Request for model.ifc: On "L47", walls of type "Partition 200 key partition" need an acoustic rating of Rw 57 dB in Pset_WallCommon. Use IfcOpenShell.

First a look at what the model holds.

```python
import ifcopenshell
import ifcopenshell.util.element

model = ifcopenshell.open("model.ifc")
print(model.schema)
storey = next(s for s in model.by_type("IfcBuildingStorey") if s.Name == "L47")
walls = [e for e in ifcopenshell.util.element.get_decomposition(storey) if e.is_a("IfcWall")]
seen = {}
for e in walls:
    element_type = ifcopenshell.util.element.get_type(e)
    key = (element_type.Name if element_type != e and element_type else None, ifcopenshell.util.element.get_pset(e, "Pset_WallCommon", "AcousticRating"))
    seen[key] = seen.get(key, 0) + 1
for (name, value), count in sorted(seen.items(), key=str):
    print(count, "x", name, "|", value)
```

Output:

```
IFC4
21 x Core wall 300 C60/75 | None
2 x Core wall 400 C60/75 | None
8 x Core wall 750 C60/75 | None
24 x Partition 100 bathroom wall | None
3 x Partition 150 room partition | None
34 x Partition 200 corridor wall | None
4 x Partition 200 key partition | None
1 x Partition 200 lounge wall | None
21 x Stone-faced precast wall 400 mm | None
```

```python
import ifcopenshell
import ifcopenshell.api.pset
import ifcopenshell.util.element

model = ifcopenshell.open("model.ifc")

storey = next(s for s in model.by_type("IfcBuildingStorey") if s.Name == "L47")
walls = [e for e in ifcopenshell.util.element.get_decomposition(storey) if e.is_a("IfcWall")]

count = 0
for e in walls:
    element_type = ifcopenshell.util.element.get_type(e)
    if element_type in (None, e) or element_type.Name != "Partition 200 key partition":
        continue
    found = ifcopenshell.util.element.get_pset(e, "Pset_WallCommon", should_inherit=False)
    if found:
        pset = model.by_id(found["id"])
        if len(ifcopenshell.util.element.get_elements_by_pset(pset)) > 1:
            pset = ifcopenshell.api.pset.unshare_pset(model, products=[e], pset=pset)[0]
    else:
        pset = ifcopenshell.api.pset.add_pset(model, product=e, name="Pset_WallCommon")
    ifcopenshell.api.pset.edit_pset(model, pset=pset, properties={"AcousticRating": "Rw 57 dB"})
    count += 1

print(count, "walls updated")

model.write("model-out.ifc")
```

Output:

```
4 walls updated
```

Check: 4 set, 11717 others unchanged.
